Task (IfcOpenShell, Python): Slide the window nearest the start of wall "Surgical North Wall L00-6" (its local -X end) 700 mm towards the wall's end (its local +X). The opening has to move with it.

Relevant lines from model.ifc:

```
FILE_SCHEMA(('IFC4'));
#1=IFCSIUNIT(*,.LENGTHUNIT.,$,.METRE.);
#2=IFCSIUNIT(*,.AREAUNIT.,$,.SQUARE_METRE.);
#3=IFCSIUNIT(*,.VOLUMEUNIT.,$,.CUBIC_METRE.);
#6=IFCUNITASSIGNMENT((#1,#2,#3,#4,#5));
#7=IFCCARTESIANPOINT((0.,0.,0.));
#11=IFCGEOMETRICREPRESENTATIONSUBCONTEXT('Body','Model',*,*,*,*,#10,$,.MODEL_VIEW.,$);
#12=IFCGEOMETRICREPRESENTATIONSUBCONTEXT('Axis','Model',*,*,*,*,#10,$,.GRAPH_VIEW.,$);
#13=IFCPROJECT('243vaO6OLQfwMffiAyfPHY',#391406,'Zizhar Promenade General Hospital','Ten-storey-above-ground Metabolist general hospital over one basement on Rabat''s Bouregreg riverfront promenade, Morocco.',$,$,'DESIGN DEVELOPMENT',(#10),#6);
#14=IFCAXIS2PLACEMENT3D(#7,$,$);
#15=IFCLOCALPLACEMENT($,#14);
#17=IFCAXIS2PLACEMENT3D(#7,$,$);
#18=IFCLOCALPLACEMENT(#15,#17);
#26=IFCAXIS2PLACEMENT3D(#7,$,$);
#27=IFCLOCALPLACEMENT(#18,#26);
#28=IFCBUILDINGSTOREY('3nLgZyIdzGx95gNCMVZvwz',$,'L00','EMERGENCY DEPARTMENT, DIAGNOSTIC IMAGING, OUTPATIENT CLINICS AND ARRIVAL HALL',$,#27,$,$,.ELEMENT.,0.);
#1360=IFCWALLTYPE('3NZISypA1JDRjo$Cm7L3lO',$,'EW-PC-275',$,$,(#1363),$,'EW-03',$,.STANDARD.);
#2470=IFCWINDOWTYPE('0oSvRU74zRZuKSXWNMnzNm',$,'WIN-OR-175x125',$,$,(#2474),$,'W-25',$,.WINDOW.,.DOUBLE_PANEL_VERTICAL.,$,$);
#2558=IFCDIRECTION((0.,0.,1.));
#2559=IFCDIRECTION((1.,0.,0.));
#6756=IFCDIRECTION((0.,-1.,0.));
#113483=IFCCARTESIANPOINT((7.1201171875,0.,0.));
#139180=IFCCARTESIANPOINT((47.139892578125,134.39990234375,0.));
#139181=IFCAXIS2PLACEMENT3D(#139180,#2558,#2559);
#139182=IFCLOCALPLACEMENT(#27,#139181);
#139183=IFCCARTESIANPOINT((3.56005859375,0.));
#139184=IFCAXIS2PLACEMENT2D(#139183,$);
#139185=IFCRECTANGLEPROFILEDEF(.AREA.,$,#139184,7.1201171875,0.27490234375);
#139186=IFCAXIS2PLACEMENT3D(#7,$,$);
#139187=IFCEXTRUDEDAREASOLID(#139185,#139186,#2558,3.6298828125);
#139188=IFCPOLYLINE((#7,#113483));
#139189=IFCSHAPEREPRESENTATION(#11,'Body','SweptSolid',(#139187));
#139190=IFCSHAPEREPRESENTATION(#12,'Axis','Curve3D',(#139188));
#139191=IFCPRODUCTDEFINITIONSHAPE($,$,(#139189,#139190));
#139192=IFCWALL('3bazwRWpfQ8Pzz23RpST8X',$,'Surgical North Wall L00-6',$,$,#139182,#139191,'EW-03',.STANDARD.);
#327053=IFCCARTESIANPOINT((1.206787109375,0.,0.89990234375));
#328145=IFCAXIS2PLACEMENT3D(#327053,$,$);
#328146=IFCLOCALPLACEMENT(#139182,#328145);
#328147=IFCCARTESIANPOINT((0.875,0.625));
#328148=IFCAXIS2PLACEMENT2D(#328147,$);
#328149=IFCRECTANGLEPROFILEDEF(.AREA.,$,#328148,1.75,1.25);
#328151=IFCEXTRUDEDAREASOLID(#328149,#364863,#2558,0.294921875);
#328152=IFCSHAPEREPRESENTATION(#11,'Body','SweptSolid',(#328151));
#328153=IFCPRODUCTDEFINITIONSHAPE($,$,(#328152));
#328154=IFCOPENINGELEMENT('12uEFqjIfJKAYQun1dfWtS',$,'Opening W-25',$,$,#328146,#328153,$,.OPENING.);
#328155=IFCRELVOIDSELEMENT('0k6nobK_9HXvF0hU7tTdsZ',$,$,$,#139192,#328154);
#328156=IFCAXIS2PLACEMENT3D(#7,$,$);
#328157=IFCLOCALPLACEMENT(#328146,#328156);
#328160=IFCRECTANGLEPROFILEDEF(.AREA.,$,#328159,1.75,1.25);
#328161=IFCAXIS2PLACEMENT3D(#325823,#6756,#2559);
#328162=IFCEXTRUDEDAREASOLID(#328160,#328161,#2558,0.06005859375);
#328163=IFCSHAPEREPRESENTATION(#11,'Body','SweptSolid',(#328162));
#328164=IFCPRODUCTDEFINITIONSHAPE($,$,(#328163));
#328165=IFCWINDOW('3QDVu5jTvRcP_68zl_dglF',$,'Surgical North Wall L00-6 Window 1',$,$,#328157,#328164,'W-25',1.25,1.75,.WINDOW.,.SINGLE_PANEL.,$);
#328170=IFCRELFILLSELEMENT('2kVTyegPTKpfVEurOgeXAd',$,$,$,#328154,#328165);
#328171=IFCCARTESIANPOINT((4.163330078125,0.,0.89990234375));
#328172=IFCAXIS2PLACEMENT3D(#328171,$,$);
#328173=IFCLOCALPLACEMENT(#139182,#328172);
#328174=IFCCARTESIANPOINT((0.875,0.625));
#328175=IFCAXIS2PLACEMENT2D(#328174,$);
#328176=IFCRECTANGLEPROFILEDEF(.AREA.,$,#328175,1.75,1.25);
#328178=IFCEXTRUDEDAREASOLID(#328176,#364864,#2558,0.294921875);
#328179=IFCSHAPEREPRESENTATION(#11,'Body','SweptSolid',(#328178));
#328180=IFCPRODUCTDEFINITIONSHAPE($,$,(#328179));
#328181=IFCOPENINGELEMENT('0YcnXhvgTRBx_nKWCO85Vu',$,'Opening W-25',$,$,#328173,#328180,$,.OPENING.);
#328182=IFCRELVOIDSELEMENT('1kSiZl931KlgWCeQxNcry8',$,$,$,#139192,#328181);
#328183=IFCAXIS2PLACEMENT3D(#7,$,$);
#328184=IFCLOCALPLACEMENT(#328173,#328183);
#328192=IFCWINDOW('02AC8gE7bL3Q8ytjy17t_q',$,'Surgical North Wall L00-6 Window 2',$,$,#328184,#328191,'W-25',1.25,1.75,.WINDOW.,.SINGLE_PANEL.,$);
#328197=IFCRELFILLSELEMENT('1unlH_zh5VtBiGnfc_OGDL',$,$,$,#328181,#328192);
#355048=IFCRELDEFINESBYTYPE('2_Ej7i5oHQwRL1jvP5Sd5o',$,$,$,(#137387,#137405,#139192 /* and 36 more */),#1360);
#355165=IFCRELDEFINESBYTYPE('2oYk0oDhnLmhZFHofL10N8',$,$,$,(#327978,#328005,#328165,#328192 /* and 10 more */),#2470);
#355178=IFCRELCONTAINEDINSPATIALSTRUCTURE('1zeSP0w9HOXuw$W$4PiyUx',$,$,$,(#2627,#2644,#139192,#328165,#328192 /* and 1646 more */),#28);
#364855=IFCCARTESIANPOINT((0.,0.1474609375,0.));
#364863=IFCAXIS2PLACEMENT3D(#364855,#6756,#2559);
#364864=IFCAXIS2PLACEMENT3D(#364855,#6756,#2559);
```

```python
import ifcopenshell
import ifcopenshell.api.geometry
import ifcopenshell.util.placement
import ifcopenshell.util.unit

model = ifcopenshell.open("model.ifc")
unit_scale = ifcopenshell.util.unit.calculate_unit_scale(model)

window = model.by_guid("3QDVu5jTvRcP_68zl_dglF")
opening = window.FillsVoids[0].RelatingOpeningElement
wall = opening.VoidsElements[0].RelatingBuildingElement

wall_matrix = ifcopenshell.util.placement.get_local_placement(wall.ObjectPlacement)
shift = wall_matrix[:3, 0] * 0.7 / unit_scale
before = ifcopenshell.util.placement.get_local_placement(window.ObjectPlacement)[:3, 3].copy()

# The window is placed relative to its opening, so it follows when the opening moves.
matrix = ifcopenshell.util.placement.get_local_placement(opening.ObjectPlacement)
matrix[:3, 3] += shift
ifcopenshell.api.geometry.edit_object_placement(
    model, product=opening, matrix=matrix, is_si=False, should_transform_children=True
)

after = ifcopenshell.util.placement.get_local_placement(window.ObjectPlacement)[:3, 3]
print("window moved by", (after - before).round(3) + 0.0)

model.write("model_updated.ifc")
```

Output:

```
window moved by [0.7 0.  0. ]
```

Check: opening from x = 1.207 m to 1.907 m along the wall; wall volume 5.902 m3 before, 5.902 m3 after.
